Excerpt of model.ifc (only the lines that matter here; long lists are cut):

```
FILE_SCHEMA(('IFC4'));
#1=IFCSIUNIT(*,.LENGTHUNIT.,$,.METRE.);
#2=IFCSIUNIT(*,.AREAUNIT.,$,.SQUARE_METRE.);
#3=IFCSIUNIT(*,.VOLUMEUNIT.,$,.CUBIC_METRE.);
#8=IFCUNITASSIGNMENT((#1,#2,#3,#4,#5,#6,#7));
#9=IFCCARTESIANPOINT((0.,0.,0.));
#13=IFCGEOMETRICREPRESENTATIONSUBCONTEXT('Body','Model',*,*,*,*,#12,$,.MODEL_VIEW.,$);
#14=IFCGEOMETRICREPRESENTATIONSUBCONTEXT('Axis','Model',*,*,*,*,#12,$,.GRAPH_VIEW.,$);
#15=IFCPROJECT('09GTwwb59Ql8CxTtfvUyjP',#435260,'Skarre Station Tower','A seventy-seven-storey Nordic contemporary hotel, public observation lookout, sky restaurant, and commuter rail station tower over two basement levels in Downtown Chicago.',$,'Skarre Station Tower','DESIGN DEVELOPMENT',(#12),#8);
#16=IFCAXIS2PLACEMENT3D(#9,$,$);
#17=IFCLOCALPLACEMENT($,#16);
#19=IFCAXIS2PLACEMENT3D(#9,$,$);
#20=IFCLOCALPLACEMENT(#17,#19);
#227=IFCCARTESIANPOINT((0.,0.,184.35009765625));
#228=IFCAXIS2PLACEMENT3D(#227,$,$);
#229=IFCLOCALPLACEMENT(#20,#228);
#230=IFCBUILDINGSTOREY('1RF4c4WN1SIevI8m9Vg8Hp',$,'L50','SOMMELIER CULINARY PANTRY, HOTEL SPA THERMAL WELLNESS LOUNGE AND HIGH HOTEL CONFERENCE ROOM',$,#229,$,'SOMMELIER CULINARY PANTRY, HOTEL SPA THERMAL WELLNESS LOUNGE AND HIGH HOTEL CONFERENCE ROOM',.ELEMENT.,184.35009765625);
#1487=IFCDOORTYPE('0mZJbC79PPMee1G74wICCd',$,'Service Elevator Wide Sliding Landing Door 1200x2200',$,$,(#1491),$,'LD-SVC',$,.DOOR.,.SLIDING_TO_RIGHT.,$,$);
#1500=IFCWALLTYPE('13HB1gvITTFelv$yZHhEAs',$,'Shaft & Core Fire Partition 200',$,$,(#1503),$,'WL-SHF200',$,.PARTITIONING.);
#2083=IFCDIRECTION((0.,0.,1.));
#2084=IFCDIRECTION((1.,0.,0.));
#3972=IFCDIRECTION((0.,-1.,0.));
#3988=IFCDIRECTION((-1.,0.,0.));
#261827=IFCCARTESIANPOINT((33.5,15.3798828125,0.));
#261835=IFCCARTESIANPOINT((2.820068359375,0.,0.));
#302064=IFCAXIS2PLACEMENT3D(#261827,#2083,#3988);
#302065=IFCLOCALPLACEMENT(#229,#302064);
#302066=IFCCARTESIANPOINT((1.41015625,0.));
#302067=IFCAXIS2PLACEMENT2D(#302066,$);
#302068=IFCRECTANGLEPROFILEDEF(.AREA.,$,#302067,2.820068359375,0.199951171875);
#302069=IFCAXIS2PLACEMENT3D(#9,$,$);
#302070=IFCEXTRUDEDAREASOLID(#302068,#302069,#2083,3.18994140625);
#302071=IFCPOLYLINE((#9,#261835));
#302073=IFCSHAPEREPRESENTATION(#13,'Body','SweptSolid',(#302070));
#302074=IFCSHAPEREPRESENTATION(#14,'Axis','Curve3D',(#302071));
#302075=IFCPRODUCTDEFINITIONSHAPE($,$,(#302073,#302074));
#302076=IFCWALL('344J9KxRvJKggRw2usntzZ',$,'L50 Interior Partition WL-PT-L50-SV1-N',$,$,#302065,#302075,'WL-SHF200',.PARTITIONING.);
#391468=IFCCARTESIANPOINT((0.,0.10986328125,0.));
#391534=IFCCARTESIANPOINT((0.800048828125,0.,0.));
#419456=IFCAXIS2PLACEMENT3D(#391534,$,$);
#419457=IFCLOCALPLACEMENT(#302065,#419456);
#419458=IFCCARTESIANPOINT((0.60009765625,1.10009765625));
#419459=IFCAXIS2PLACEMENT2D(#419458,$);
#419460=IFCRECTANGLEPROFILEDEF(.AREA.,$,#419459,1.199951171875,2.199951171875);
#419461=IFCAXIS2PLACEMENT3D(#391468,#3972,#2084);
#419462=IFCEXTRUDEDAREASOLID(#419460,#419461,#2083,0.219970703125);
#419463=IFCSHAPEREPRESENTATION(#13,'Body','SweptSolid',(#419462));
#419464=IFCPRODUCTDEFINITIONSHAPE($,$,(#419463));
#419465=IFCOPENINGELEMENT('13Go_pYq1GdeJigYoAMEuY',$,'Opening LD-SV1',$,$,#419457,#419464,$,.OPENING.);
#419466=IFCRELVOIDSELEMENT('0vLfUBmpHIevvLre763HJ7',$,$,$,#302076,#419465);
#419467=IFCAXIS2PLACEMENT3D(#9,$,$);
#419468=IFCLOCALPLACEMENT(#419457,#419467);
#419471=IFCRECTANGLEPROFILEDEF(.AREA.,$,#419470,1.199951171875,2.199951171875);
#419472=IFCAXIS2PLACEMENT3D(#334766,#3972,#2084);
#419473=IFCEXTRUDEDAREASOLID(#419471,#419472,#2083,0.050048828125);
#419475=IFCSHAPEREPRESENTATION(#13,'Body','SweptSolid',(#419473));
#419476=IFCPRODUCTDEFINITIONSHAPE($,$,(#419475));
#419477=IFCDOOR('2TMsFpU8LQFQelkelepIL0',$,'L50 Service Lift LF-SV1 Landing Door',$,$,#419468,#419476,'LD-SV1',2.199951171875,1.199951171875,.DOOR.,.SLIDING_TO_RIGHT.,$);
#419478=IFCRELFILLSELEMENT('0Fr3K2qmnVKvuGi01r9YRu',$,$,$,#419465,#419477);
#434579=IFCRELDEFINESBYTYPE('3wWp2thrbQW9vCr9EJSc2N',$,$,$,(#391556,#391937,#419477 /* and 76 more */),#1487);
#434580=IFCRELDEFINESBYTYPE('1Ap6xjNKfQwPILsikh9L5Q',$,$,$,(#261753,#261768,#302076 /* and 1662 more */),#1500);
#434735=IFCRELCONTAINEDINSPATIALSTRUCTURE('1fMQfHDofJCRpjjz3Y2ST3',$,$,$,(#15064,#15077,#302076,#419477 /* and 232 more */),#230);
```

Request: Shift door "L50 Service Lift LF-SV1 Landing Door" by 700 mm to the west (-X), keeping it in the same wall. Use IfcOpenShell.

```python
import ifcopenshell
import ifcopenshell.api.geometry
import ifcopenshell.util.placement
import ifcopenshell.util.unit

model = ifcopenshell.open("model.ifc")
unit_scale = ifcopenshell.util.unit.calculate_unit_scale(model)

door = model.by_id(419477)
opening = door.FillsVoids[0].RelatingOpeningElement
wall = opening.VoidsElements[0].RelatingBuildingElement

wall_matrix = ifcopenshell.util.placement.get_local_placement(wall.ObjectPlacement)
shift = wall_matrix[:3, 0] * 0.7 / unit_scale
before = ifcopenshell.util.placement.get_local_placement(door.ObjectPlacement)[:3, 3].copy()

# The door is placed relative to its opening, so it follows when the opening moves.
matrix = ifcopenshell.util.placement.get_local_placement(opening.ObjectPlacement)
matrix[:3, 3] += shift
ifcopenshell.api.geometry.edit_object_placement(
    model, product=opening, matrix=matrix, is_si=False, should_transform_children=True
)

after = ifcopenshell.util.placement.get_local_placement(door.ObjectPlacement)[:3, 3]
print("door moved by", (after - before).round(3) + 0.0)

model.write("model_edited.ifc")
```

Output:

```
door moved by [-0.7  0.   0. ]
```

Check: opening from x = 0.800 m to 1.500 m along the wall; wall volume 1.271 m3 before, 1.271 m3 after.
